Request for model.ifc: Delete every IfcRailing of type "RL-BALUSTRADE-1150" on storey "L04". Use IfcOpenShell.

First a look at what the model holds.

```python
import ifcopenshell
import ifcopenshell.util.element

model = ifcopenshell.open("model.ifc")
print(model.schema)
storey = next(s for s in model.by_type("IfcBuildingStorey") if s.Name == "L04")
railings = [e for e in ifcopenshell.util.element.get_decomposition(storey) if e.is_a("IfcRailing")]
seen = {}
for e in railings:
    element_type = ifcopenshell.util.element.get_type(e)
    name = element_type.Name if element_type not in (None, e) else None
    seen[name] = seen.get(name, 0) + 1
for name, count in sorted(seen.items(), key=str):
    print(count, "x", name)
```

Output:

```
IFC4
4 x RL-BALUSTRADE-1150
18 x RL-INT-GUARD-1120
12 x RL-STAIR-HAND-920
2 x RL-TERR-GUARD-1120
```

```python
import ifcopenshell
import ifcopenshell.api.root
import ifcopenshell.util.element

model = ifcopenshell.open("model.ifc")

storey = next(s for s in model.by_type("IfcBuildingStorey") if s.Name == "L04")
railings = [e for e in ifcopenshell.util.element.get_decomposition(storey) if e.is_a("IfcRailing")]
targets = [e for e in railings if (t := ifcopenshell.util.element.get_type(e)) not in (None, e) and t.Name == "RL-BALUSTRADE-1150"]

for e in targets:
    ifcopenshell.api.root.remove_product(model, product=e)
print(len(targets), "removed")

model.write("model_rev.ifc")
```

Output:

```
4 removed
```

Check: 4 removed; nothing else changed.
